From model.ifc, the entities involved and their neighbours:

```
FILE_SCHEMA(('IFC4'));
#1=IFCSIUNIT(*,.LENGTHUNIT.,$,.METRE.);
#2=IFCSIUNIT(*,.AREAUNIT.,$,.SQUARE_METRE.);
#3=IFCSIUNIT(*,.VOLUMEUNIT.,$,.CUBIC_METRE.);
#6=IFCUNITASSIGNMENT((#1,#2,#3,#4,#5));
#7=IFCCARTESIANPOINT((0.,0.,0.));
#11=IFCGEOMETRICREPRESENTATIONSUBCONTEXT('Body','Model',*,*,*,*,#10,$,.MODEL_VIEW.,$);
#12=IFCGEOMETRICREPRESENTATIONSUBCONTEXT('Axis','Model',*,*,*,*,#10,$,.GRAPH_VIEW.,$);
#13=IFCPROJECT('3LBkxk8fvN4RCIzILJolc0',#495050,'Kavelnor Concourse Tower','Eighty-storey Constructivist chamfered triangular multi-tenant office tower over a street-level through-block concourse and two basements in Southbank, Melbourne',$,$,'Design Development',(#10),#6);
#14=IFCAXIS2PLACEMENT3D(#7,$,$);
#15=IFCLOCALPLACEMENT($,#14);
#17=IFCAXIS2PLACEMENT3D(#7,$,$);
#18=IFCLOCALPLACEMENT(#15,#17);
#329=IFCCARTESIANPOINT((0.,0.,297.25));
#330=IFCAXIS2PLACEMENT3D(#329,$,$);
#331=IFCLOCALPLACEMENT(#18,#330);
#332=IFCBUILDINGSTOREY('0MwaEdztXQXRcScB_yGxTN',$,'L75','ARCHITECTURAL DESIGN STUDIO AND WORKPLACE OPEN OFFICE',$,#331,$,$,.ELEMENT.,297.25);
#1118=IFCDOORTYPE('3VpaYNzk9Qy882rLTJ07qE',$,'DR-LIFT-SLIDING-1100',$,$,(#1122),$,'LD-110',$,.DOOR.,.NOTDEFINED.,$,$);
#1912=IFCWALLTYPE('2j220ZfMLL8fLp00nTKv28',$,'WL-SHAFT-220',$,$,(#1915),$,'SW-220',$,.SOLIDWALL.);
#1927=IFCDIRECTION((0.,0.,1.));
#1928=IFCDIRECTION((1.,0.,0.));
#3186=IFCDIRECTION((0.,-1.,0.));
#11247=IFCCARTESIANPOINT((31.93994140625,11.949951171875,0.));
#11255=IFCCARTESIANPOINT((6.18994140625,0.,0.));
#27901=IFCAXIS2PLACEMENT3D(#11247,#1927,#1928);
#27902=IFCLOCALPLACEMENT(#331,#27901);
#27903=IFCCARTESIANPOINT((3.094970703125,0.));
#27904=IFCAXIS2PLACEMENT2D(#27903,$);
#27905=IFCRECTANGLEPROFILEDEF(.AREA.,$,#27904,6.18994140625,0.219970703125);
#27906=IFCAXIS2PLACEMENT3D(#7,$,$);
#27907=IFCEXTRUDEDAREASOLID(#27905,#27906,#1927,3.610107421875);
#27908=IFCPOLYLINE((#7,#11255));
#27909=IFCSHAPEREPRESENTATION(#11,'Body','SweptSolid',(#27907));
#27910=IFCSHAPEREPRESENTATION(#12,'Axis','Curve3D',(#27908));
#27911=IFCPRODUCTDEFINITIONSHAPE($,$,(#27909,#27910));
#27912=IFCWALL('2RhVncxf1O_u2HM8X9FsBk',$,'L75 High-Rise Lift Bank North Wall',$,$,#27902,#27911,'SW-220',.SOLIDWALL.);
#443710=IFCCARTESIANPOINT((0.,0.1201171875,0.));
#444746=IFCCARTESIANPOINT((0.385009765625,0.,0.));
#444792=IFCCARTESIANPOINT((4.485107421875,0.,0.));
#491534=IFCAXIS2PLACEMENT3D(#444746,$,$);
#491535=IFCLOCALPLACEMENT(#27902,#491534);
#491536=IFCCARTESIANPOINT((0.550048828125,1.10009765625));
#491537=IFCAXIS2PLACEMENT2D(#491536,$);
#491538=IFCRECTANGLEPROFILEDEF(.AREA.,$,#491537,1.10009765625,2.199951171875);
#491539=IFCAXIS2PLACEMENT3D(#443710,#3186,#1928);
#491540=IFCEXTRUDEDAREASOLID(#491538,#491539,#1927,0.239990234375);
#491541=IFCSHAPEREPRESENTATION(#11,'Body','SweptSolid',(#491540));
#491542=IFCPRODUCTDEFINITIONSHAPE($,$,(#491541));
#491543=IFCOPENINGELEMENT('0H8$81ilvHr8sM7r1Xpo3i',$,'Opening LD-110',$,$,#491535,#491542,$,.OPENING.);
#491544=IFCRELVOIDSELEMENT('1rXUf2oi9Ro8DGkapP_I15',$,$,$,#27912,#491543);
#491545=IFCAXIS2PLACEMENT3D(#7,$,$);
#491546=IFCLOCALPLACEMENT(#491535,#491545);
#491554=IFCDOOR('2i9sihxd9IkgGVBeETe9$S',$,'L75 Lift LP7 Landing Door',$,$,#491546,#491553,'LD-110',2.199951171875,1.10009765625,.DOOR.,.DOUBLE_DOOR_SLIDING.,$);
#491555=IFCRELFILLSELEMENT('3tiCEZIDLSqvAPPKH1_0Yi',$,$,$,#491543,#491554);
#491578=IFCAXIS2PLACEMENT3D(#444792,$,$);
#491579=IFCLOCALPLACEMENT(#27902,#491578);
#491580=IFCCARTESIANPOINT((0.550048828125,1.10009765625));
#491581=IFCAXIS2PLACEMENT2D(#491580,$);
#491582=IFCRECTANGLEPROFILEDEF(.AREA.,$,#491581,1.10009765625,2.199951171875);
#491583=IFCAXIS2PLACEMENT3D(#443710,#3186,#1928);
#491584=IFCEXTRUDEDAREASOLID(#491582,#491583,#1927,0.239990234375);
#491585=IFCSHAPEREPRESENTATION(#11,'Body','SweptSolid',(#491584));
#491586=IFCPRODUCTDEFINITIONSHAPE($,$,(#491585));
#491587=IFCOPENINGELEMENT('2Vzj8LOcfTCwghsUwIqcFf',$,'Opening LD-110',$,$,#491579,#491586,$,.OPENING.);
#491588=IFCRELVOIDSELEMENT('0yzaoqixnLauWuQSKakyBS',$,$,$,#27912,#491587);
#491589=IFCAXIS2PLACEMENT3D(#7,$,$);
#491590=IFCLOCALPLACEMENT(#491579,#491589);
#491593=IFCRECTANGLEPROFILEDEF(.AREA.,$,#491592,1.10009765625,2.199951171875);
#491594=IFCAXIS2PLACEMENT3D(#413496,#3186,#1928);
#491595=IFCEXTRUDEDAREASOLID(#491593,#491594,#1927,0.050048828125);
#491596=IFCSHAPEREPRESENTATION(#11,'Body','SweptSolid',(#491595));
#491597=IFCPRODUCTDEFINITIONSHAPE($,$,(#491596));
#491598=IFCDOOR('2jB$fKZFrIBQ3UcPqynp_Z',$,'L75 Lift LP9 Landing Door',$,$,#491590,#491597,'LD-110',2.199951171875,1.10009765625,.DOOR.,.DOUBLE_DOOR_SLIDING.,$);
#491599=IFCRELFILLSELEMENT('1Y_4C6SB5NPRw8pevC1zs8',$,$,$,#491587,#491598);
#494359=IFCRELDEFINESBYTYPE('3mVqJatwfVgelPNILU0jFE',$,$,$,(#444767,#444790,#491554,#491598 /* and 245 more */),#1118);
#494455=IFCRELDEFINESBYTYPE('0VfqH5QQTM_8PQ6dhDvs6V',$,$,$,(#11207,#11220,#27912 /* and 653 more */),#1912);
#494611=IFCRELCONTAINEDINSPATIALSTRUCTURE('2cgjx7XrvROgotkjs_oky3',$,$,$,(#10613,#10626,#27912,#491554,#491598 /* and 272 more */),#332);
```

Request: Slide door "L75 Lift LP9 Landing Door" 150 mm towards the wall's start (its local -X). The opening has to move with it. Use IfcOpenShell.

```python
import ifcopenshell
import ifcopenshell.api.geometry
import ifcopenshell.util.placement

model = ifcopenshell.open("model.ifc")

door = model.by_guid("2jB$fKZFrIBQ3UcPqynp_Z")
opening = door.FillsVoids[0].RelatingOpeningElement
wall = opening.VoidsElements[0].RelatingBuildingElement

wall_matrix = ifcopenshell.util.placement.get_local_placement(wall.ObjectPlacement)
shift = wall_matrix[:3, 0] * -0.15
before = ifcopenshell.util.placement.get_local_placement(door.ObjectPlacement)[:3, 3].copy()

# The door is placed relative to its opening, so it follows when the opening moves.
matrix = ifcopenshell.util.placement.get_local_placement(opening.ObjectPlacement)
matrix[:3, 3] += shift
ifcopenshell.api.geometry.edit_object_placement(
    model, product=opening, matrix=matrix, is_si=False, should_transform_children=True
)

after = ifcopenshell.util.placement.get_local_placement(door.ObjectPlacement)[:3, 3]
print("door moved by", (after - before).round(3) + 0.0)

model.write("model_updated.ifc")
```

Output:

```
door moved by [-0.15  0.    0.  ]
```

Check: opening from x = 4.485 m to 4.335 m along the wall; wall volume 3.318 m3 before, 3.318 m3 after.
